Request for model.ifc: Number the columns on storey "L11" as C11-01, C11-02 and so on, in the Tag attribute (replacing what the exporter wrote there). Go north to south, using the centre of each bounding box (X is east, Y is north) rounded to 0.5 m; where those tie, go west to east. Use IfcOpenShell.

First a look at what the model holds.

```python
import ifcopenshell
import ifcopenshell.util.element
import ifcopenshell.util.placement

model = ifcopenshell.open("model.ifc")
print(model.schema)
storey = next(s for s in model.by_type("IfcBuildingStorey") if s.Name == "L11")
columns = [e for e in ifcopenshell.util.element.get_decomposition(storey) if e.is_a("IfcColumn")]
for e in sorted(columns, key=lambda e: e.id()):
    origin = ifcopenshell.util.placement.get_local_placement(e.ObjectPlacement)[:3, 3]
    print(e.id(), e.Tag, e.Name, origin.round(2) + 0.0, sep=" | ")
```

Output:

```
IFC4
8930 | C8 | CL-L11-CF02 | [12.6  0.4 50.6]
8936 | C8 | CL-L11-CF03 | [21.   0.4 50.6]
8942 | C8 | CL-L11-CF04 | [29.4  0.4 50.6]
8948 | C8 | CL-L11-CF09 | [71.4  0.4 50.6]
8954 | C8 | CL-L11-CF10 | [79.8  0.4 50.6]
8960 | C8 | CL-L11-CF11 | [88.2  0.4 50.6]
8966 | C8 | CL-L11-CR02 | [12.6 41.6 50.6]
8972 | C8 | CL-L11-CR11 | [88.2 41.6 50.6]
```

```python
import ifcopenshell
import ifcopenshell.geom
import ifcopenshell.util.element
import ifcopenshell.util.shape

model = ifcopenshell.open("model.ifc")
settings = ifcopenshell.geom.settings()
settings.set("use-world-coords", True)


def centre(element):
    shape = ifcopenshell.geom.create_shape(settings, element)
    return ifcopenshell.util.shape.get_bbox_centroid(shape.geometry)


storey = next(s for s in model.by_type("IfcBuildingStorey") if s.Name == "L11")
columns = [e for e in ifcopenshell.util.element.get_decomposition(storey) if e.is_a("IfcColumn")]

# Insertion points can sit at a corner or the storey origin, so sort by the geometry (in metres).
centres = {e: centre(e) for e in columns}
columns.sort(key=lambda e: (-round(centres[e][1] / 0.5), centres[e][0]))

for i, e in enumerate(columns, start=1):
    number = f"C11-{i:02d}"
    e.Tag = number
    print(e.id(), number)

model.write("model_edited.ifc")
```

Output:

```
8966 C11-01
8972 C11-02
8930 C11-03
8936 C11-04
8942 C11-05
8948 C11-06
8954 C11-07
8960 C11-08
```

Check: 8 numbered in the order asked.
